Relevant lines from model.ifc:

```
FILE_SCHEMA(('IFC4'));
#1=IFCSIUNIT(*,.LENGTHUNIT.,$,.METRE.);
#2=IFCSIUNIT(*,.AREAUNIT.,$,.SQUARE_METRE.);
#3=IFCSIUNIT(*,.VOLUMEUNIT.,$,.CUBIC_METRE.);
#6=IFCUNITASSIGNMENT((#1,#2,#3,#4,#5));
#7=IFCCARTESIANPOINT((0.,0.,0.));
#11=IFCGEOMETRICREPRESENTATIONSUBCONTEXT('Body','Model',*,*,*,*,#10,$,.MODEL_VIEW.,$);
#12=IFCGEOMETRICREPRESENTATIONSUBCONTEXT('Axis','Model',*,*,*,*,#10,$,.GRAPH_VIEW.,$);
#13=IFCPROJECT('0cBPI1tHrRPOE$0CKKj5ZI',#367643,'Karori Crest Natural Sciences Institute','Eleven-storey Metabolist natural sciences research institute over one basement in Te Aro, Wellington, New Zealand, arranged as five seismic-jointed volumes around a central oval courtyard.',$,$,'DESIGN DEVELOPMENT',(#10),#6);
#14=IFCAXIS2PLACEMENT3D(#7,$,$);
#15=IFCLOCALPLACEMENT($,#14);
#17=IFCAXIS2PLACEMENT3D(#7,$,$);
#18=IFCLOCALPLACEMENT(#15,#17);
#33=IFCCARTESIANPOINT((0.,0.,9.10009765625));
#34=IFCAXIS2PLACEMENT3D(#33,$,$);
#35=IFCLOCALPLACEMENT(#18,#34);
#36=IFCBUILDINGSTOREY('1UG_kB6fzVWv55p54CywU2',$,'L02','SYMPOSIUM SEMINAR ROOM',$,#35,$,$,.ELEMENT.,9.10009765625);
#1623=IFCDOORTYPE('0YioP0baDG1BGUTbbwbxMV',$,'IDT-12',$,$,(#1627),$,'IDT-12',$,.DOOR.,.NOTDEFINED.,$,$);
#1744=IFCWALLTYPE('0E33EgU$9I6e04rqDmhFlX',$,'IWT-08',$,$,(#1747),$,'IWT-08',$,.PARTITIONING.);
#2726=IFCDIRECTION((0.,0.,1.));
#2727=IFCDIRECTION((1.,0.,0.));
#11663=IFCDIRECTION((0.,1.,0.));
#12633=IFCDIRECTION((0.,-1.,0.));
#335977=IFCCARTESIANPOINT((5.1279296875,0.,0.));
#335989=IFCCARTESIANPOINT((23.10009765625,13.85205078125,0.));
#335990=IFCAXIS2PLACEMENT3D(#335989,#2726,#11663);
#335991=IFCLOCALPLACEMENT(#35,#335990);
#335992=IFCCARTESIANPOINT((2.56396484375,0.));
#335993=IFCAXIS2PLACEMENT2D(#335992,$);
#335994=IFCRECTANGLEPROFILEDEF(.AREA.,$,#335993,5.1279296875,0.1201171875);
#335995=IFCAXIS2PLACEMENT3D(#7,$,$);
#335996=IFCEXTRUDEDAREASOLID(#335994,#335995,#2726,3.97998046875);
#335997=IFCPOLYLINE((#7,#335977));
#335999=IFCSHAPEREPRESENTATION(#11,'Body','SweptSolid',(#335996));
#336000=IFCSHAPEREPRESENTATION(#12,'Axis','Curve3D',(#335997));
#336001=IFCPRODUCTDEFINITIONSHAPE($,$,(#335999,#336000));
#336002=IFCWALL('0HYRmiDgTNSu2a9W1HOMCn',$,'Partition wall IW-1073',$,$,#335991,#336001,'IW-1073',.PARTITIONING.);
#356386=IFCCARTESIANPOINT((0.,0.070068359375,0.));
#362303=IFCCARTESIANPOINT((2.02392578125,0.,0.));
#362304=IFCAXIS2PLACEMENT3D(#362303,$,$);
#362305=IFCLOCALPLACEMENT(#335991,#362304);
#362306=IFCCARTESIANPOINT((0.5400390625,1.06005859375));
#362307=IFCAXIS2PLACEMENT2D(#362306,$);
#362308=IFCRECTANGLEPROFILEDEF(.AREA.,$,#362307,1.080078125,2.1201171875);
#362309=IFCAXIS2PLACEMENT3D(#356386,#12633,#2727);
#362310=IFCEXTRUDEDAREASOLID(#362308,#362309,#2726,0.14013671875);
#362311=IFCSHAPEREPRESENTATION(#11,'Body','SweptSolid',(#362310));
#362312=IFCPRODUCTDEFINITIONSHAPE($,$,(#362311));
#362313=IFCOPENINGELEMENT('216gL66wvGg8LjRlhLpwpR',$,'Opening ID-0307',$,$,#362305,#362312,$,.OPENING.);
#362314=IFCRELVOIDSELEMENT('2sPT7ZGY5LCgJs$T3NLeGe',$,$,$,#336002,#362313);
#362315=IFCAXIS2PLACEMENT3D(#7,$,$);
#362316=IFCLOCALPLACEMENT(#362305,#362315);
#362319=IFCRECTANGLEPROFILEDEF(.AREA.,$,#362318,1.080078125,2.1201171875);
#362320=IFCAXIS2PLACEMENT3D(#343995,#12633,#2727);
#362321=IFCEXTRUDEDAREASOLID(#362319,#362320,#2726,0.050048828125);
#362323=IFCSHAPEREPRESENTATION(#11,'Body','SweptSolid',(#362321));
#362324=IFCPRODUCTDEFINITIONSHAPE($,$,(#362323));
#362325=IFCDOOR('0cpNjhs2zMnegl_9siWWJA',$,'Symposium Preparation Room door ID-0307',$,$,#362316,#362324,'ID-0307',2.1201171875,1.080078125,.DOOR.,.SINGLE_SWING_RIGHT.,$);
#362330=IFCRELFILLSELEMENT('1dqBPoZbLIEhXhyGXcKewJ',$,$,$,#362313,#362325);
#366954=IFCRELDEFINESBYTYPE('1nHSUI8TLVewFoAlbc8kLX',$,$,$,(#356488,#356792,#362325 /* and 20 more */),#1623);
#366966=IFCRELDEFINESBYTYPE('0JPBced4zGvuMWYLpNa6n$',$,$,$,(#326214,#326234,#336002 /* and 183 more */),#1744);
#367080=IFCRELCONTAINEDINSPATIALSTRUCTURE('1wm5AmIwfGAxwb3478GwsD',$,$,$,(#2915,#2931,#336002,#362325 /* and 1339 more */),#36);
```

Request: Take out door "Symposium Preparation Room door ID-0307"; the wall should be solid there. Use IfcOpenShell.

```python
import ifcopenshell
import ifcopenshell.api.feature
import ifcopenshell.api.root
import ifcopenshell.geom
import ifcopenshell.util.shape

model = ifcopenshell.open("model.ifc")
settings = ifcopenshell.geom.settings()


def volume(element):
    """Net volume in cubic metres, openings subtracted."""
    shape = ifcopenshell.geom.create_shape(settings, element)
    return ifcopenshell.util.shape.get_volume(shape.geometry)


door = model.by_guid("0cpNjhs2zMnegl_9siWWJA")
opening = door.FillsVoids[0].RelatingOpeningElement
wall = opening.VoidsElements[0].RelatingBuildingElement
before = volume(wall)

ifcopenshell.api.root.remove_product(model, product=door)
ifcopenshell.api.feature.remove_feature(model, feature=opening)

after = volume(wall)

print(f"wall volume {before:.3f} -> {after:.3f} m3")

model.write("model_updated.ifc")
```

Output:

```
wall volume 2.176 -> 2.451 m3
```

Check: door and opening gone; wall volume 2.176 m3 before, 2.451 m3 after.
